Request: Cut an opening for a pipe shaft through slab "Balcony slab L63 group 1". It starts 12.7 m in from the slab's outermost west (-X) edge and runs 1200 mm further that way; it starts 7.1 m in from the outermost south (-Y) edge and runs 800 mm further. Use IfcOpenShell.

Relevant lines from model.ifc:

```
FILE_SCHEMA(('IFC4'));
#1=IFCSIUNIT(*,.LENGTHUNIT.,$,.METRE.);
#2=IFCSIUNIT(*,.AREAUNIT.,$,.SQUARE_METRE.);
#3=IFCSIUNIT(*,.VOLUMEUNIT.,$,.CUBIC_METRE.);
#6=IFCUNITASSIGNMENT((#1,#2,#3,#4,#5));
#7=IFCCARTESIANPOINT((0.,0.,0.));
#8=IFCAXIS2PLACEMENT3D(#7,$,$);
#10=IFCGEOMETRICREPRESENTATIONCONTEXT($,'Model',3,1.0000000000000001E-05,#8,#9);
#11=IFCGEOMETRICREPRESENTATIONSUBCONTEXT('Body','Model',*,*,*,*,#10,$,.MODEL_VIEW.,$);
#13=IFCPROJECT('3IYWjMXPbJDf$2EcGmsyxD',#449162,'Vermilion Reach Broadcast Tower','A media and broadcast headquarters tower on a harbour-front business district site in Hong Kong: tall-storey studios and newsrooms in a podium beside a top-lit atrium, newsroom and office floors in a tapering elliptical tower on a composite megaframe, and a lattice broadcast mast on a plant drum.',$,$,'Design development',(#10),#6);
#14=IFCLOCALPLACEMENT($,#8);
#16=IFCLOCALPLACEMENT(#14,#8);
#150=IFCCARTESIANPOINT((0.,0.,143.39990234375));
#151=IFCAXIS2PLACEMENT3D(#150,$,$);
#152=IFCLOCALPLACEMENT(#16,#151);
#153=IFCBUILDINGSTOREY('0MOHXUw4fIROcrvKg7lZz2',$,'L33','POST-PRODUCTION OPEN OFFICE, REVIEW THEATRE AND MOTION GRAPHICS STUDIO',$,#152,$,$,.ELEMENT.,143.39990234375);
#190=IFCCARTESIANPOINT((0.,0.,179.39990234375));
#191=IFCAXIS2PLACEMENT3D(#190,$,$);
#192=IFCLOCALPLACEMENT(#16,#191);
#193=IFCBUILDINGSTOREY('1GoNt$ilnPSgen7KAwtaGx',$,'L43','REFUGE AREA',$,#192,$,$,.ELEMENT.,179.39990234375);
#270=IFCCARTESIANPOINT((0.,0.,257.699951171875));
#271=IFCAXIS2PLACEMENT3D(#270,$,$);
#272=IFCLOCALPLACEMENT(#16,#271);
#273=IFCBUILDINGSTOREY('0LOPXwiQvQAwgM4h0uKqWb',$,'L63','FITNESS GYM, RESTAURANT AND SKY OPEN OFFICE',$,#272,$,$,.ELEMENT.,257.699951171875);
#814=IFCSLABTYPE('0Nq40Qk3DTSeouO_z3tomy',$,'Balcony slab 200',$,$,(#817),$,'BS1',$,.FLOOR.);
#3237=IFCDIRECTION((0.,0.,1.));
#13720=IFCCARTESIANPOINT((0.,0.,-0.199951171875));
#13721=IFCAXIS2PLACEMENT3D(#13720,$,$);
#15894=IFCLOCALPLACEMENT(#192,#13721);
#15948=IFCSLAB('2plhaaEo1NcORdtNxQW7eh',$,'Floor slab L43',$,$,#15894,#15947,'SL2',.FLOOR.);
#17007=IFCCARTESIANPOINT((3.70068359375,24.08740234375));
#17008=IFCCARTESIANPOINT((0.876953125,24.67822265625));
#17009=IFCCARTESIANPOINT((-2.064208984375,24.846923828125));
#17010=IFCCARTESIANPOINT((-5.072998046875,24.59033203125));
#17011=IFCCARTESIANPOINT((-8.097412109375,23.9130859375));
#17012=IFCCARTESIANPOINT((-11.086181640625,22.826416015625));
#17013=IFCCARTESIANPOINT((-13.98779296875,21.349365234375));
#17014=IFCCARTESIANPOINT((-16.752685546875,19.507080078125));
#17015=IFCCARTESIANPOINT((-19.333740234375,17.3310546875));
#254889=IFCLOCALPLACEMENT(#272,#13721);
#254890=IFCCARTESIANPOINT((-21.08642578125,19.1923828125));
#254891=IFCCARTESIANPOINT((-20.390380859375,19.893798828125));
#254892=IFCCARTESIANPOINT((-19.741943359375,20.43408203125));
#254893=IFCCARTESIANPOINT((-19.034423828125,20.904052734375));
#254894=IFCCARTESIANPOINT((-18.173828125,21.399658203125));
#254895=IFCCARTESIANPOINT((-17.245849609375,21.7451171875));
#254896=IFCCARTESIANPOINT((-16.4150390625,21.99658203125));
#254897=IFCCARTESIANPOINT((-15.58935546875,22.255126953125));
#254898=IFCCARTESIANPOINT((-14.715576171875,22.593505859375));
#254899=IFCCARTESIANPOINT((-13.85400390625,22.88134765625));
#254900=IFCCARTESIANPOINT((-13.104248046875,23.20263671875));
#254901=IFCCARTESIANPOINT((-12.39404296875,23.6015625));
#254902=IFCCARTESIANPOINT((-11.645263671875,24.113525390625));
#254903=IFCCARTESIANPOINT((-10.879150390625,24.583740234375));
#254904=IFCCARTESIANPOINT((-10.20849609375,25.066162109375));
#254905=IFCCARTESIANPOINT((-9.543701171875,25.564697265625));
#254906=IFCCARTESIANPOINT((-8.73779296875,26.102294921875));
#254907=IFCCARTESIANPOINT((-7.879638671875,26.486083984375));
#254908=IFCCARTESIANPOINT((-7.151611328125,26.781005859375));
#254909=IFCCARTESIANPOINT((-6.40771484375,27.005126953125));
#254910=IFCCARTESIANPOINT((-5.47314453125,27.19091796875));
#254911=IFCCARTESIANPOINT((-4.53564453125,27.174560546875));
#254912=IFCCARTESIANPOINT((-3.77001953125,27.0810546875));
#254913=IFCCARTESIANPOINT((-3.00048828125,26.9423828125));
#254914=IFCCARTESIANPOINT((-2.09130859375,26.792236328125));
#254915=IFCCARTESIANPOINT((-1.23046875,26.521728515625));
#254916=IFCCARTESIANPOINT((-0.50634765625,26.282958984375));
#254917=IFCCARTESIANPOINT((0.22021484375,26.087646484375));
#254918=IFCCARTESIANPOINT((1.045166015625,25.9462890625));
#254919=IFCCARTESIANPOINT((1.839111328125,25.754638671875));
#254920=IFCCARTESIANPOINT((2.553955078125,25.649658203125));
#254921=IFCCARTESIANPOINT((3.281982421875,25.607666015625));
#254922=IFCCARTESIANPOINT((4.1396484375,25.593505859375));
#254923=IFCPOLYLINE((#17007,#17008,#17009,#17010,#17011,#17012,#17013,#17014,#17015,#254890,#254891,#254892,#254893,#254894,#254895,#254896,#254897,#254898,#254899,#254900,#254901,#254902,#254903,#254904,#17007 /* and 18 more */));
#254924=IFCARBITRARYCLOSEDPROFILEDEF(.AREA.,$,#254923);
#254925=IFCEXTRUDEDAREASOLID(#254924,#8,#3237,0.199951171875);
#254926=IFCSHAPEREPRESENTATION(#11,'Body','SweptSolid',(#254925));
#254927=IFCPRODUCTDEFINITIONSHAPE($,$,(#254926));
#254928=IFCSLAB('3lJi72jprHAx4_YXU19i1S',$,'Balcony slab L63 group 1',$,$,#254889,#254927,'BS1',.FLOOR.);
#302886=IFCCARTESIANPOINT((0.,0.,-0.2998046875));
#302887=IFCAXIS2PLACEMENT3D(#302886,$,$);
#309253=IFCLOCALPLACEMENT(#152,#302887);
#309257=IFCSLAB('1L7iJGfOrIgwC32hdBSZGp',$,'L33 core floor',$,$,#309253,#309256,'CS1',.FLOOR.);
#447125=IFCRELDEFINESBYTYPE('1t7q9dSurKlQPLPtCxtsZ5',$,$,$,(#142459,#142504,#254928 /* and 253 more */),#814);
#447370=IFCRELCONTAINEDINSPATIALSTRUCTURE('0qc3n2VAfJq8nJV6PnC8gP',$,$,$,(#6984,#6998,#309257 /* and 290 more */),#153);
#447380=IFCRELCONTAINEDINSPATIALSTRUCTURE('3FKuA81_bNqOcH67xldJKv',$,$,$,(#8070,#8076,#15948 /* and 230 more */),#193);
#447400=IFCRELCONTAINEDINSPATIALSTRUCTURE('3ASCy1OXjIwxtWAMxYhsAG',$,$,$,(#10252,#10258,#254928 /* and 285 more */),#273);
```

```python
import numpy as np
import ifcopenshell
import ifcopenshell.api.feature
import ifcopenshell.api.geometry
import ifcopenshell.api.root
import ifcopenshell.geom
import ifcopenshell.util.placement
import ifcopenshell.util.representation
import ifcopenshell.util.shape
import ifcopenshell.util.unit

model = ifcopenshell.open("model.ifc")
unit_scale = ifcopenshell.util.unit.calculate_unit_scale(model)
settings = ifcopenshell.geom.settings()


def volume(element):
    """Net volume in cubic metres, openings subtracted."""
    shape = ifcopenshell.geom.create_shape(settings, element)
    return ifcopenshell.util.shape.get_volume(shape.geometry)


slab = model.by_guid("3lJi72jprHAx4_YXU19i1S")
before = volume(slab)

# Extent in the slab's own axes, in metres. The edges named are its -X and -Y sides.
slab_shape = ifcopenshell.geom.create_shape(settings, slab)
vertices = ifcopenshell.util.shape.get_vertices(slab_shape.geometry)
x_min, y_min, bottom = vertices.min(axis=0)
top = vertices[:, 2].max()

opening = ifcopenshell.api.root.create_entity(model, ifc_class="IfcOpeningElement", name="Pipe shaft opening", predefined_type="OPENING")
context = ifcopenshell.util.representation.get_context(model, "Model", "Body", "MODEL_VIEW")
width, depth = 1.2, 0.8
outline = [(0.0, 0.0), (width, 0.0), (width, depth), (0.0, depth), (0.0, 0.0)]
# Overshoot both faces by 50 mm so the cut is clean.
shape = ifcopenshell.api.geometry.add_slab_representation(
    model, context=context, depth=top - bottom + 0.1, polyline=outline
)
ifcopenshell.api.geometry.assign_representation(model, product=opening, representation=shape)

matrix = ifcopenshell.util.placement.get_local_placement(slab.ObjectPlacement)
matrix[:, 3] = matrix @ np.append(np.array([x_min + 12.7, y_min + 7.1, bottom - 0.05]) / unit_scale, 1.0)
ifcopenshell.api.geometry.edit_object_placement(model, product=opening, matrix=matrix, is_si=False)
ifcopenshell.api.feature.add_feature(model, feature=opening, element=slab)

after = volume(slab)

print(f"slab volume {before:.3f} -> {after:.3f} m3")

model.write("model_updated.ifc")
```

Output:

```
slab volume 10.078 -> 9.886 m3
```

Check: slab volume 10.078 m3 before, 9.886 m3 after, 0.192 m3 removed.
